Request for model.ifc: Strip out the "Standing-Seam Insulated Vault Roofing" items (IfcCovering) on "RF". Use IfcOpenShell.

First a look at what the model holds.

```python
import ifcopenshell
import ifcopenshell.util.element

model = ifcopenshell.open("model.ifc")
print(model.schema)
storey = next(s for s in model.by_type("IfcBuildingStorey") if s.Name == "RF")
coverings = [e for e in ifcopenshell.util.element.get_decomposition(storey) if e.is_a("IfcCovering")]
seen = {}
for e in coverings:
    element_type = ifcopenshell.util.element.get_type(e)
    name = element_type.Name if element_type not in (None, e) else None
    seen[name] = seen.get(name, 0) + 1
for name, count in sorted(seen.items(), key=str):
    print(count, "x", name)
```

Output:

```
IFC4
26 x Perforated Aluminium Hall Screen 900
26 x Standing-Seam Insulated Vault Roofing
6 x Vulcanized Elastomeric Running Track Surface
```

```python
import ifcopenshell
import ifcopenshell.api.root
import ifcopenshell.util.element

model = ifcopenshell.open("model.ifc")

storey = next(s for s in model.by_type("IfcBuildingStorey") if s.Name == "RF")
coverings = [e for e in ifcopenshell.util.element.get_decomposition(storey) if e.is_a("IfcCovering")]
targets = [e for e in coverings if (t := ifcopenshell.util.element.get_type(e)) not in (None, e) and t.Name == "Standing-Seam Insulated Vault Roofing"]

for e in targets:
    ifcopenshell.api.root.remove_product(model, product=e)
print(len(targets), "removed")

model.write("model_updated.ifc")
```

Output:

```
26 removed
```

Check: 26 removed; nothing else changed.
